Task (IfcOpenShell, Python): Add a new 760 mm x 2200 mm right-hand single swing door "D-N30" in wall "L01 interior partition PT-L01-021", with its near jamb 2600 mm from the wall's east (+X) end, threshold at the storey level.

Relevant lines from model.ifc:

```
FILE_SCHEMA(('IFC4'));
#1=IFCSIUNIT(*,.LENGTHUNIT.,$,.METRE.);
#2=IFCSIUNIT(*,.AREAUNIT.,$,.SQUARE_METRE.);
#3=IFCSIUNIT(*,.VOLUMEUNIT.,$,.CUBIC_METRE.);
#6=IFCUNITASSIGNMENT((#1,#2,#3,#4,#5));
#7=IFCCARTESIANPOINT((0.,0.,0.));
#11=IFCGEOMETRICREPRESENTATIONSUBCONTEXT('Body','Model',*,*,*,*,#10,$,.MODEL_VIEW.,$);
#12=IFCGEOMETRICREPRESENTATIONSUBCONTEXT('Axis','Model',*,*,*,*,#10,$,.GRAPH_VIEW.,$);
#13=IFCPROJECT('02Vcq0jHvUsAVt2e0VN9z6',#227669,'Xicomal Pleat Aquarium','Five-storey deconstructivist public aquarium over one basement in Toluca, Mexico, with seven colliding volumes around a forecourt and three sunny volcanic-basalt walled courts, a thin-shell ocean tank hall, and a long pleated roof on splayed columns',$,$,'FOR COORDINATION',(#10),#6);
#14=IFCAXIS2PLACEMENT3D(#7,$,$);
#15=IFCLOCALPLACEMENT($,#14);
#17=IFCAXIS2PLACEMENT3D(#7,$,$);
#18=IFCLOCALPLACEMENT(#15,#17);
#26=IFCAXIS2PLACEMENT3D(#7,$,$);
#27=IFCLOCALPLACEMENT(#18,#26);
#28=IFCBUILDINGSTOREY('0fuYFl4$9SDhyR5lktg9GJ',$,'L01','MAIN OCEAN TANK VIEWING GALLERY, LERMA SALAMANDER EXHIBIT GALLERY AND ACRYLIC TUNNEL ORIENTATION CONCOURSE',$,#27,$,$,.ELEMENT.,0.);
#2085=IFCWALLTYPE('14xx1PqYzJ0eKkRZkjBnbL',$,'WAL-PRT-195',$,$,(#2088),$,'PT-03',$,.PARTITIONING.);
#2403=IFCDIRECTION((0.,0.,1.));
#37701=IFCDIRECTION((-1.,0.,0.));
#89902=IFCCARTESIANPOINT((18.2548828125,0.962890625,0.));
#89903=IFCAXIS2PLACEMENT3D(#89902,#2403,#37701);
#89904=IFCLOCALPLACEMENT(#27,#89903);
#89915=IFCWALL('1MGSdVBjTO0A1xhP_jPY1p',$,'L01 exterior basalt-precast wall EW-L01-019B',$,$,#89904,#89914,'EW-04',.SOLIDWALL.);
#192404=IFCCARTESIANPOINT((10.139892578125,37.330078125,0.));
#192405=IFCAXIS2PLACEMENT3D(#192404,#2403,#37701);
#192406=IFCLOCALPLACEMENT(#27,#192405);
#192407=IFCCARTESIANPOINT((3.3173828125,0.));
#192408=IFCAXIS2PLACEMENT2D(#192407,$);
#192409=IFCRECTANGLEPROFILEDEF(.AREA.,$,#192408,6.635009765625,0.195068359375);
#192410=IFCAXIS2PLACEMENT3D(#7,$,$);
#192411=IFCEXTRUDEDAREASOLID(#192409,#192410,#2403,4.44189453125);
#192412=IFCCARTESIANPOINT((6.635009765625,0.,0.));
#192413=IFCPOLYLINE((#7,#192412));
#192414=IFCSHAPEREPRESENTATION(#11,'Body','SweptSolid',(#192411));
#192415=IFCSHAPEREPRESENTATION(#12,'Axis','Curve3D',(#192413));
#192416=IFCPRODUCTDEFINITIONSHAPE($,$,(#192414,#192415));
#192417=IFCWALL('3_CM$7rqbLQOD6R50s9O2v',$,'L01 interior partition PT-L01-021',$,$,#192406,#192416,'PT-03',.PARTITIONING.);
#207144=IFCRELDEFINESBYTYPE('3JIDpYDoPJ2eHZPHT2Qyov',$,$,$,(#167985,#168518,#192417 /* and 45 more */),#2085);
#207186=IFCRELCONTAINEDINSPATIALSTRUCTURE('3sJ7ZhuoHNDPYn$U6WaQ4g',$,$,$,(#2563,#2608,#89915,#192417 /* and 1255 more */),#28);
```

```python
import numpy as np
import ifcopenshell
import ifcopenshell.api.feature
import ifcopenshell.api.geometry
import ifcopenshell.api.root
import ifcopenshell.api.spatial
import ifcopenshell.geom
import ifcopenshell.util.element
import ifcopenshell.util.placement
import ifcopenshell.util.representation
import ifcopenshell.util.shape
import ifcopenshell.util.unit

model = ifcopenshell.open("model.ifc")
unit_scale = ifcopenshell.util.unit.calculate_unit_scale(model)
settings = ifcopenshell.geom.settings()


def volume(element):
    """Net volume in cubic metres, openings subtracted."""
    shape = ifcopenshell.geom.create_shape(settings, element)
    return ifcopenshell.util.shape.get_volume(shape.geometry)


wall = model.by_guid("3_CM$7rqbLQOD6R50s9O2v")
storey = ifcopenshell.util.element.get_container(wall, ifc_class="IfcBuildingStorey")
context = ifcopenshell.util.representation.get_context(model, "Model", "Body", "MODEL_VIEW")
before = volume(wall)

width, height, from_end, sill = 0.76, 2.2, 2.6, 0.0  # metres

# The wall runs along its own X axis, and the end named is its -X end.
wall_shape = ifcopenshell.geom.create_shape(settings, wall)
x, y, z = ifcopenshell.util.shape.get_vertices(wall_shape.geometry).T
start = x.min() + from_end
face, thickness = float(y.min()), float(y.max() - y.min())
wall_matrix = ifcopenshell.util.placement.get_local_placement(wall.ObjectPlacement)
level = ifcopenshell.util.placement.get_local_placement(storey.ObjectPlacement)[2, 3]


def in_wall(x, y):
    """Placement at x, y metres in the wall's axes, at sill height."""
    matrix = wall_matrix.copy()
    matrix[:, 3] = wall_matrix @ np.array([x / unit_scale, y / unit_scale, 0.0, 1.0])
    matrix[2, 3] = level + sill / unit_scale
    return matrix


# Opening: a box that overshoots both wall faces by 50 mm.
opening = ifcopenshell.api.root.create_entity(model, ifc_class="IfcOpeningElement", predefined_type="OPENING")
box = ifcopenshell.api.geometry.add_wall_representation(
    model, context=context, length=width, height=height, thickness=thickness + 0.1
)
ifcopenshell.api.geometry.assign_representation(model, product=opening, representation=box)
ifcopenshell.api.geometry.edit_object_placement(model, product=opening, matrix=in_wall(start, face - 0.05), is_si=False)
ifcopenshell.api.feature.add_feature(model, feature=opening, element=wall)

door = ifcopenshell.api.root.create_entity(model, ifc_class="IfcDoor", name="D-N30", predefined_type="DOOR")
door.OverallWidth, door.OverallHeight = width / unit_scale, height / unit_scale
door.OperationType = "SINGLE_SWING_RIGHT"
body = ifcopenshell.api.geometry.add_door_representation(
    model,
    context=context,
    overall_width=door.OverallWidth,
    overall_height=door.OverallHeight,
    operation_type="SINGLE_SWING_RIGHT",
    lining_properties={"LiningDepth": thickness / unit_scale, "ThresholdDepth": thickness / unit_scale},
)
ifcopenshell.api.geometry.assign_representation(model, product=door, representation=body)
ifcopenshell.api.spatial.assign_container(model, products=[door], relating_structure=storey)
ifcopenshell.api.feature.add_filling(model, opening=opening, element=door)

# The lining spans the wall, so the door starts at the wall face.
ifcopenshell.api.geometry.edit_object_placement(model, product=door, matrix=in_wall(start, face), is_si=False)

after = volume(wall)

print(f"wall volume {before:.3f} -> {after:.3f} m3")

model.write("model_updated.ifc")
```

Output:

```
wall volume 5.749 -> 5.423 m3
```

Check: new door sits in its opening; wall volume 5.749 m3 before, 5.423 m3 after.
